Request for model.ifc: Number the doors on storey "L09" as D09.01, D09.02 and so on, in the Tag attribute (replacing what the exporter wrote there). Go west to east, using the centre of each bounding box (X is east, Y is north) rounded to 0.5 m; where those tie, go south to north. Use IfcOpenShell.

First a look at what the model holds.

```python
import ifcopenshell
import ifcopenshell.util.element
import ifcopenshell.util.placement

model = ifcopenshell.open("model.ifc")
print(model.schema)
storey = next(s for s in model.by_type("IfcBuildingStorey") if s.Name == "L09")
doors = [e for e in ifcopenshell.util.element.get_decomposition(storey) if e.is_a("IfcDoor")]
for e in sorted(doors, key=lambda e: e.id()):
    origin = ifcopenshell.util.placement.get_local_placement(e.ObjectPlacement)[:3, 3]
    print(e.id(), e.Tag, e.Name, origin.round(2) + 0.0, sep=" | ")
```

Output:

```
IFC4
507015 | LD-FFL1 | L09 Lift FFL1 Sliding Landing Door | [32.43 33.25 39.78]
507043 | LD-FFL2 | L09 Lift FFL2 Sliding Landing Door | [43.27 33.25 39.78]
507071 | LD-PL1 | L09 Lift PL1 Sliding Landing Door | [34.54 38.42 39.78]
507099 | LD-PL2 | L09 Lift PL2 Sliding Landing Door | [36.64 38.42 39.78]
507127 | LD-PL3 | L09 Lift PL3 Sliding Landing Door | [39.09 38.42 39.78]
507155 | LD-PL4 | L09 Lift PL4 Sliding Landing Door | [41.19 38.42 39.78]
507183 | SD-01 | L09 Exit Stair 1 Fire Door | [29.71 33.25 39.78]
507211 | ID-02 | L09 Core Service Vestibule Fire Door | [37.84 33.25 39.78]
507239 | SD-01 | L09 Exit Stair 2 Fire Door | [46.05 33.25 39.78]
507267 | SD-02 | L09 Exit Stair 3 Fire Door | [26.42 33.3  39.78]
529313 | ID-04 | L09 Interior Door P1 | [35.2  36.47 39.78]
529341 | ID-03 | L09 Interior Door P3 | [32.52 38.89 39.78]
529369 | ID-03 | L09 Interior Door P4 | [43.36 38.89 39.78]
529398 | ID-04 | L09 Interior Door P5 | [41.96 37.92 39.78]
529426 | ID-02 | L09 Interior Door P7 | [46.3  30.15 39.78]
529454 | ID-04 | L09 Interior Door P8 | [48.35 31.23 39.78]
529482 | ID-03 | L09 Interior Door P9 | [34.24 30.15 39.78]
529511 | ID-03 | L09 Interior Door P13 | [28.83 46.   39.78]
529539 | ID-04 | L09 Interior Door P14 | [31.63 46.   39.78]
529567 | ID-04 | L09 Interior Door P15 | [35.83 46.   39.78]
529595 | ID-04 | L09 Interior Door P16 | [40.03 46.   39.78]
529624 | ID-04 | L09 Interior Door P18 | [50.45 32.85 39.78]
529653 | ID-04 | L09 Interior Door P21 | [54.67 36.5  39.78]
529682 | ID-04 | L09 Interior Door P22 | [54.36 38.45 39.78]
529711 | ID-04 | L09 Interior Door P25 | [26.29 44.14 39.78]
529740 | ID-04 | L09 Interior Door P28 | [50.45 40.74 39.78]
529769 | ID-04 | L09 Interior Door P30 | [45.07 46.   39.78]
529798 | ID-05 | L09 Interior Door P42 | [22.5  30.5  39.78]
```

```python
import ifcopenshell
import ifcopenshell.geom
import ifcopenshell.util.element
import ifcopenshell.util.shape

model = ifcopenshell.open("model.ifc")
settings = ifcopenshell.geom.settings()
settings.set("use-world-coords", True)


def centre(element):
    shape = ifcopenshell.geom.create_shape(settings, element)
    return ifcopenshell.util.shape.get_bbox_centroid(shape.geometry)


storey = next(s for s in model.by_type("IfcBuildingStorey") if s.Name == "L09")
doors = [e for e in ifcopenshell.util.element.get_decomposition(storey) if e.is_a("IfcDoor")]

# Insertion points can sit at a corner or the storey origin, so sort by the geometry (in metres).
centres = {e: centre(e) for e in doors}
doors.sort(key=lambda e: (round(centres[e][0] / 0.5), centres[e][1]))

for i, e in enumerate(doors, start=1):
    number = f"D09.{i:02d}"
    e.Tag = number
    print(e.id(), number)

model.write("model-out.ifc")
```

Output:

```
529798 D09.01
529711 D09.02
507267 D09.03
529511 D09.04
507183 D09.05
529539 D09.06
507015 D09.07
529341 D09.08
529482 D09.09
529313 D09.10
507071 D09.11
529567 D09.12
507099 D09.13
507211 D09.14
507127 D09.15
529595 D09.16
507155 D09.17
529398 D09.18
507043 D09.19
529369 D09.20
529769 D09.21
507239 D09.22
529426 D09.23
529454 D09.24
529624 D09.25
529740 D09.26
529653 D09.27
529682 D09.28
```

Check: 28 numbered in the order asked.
